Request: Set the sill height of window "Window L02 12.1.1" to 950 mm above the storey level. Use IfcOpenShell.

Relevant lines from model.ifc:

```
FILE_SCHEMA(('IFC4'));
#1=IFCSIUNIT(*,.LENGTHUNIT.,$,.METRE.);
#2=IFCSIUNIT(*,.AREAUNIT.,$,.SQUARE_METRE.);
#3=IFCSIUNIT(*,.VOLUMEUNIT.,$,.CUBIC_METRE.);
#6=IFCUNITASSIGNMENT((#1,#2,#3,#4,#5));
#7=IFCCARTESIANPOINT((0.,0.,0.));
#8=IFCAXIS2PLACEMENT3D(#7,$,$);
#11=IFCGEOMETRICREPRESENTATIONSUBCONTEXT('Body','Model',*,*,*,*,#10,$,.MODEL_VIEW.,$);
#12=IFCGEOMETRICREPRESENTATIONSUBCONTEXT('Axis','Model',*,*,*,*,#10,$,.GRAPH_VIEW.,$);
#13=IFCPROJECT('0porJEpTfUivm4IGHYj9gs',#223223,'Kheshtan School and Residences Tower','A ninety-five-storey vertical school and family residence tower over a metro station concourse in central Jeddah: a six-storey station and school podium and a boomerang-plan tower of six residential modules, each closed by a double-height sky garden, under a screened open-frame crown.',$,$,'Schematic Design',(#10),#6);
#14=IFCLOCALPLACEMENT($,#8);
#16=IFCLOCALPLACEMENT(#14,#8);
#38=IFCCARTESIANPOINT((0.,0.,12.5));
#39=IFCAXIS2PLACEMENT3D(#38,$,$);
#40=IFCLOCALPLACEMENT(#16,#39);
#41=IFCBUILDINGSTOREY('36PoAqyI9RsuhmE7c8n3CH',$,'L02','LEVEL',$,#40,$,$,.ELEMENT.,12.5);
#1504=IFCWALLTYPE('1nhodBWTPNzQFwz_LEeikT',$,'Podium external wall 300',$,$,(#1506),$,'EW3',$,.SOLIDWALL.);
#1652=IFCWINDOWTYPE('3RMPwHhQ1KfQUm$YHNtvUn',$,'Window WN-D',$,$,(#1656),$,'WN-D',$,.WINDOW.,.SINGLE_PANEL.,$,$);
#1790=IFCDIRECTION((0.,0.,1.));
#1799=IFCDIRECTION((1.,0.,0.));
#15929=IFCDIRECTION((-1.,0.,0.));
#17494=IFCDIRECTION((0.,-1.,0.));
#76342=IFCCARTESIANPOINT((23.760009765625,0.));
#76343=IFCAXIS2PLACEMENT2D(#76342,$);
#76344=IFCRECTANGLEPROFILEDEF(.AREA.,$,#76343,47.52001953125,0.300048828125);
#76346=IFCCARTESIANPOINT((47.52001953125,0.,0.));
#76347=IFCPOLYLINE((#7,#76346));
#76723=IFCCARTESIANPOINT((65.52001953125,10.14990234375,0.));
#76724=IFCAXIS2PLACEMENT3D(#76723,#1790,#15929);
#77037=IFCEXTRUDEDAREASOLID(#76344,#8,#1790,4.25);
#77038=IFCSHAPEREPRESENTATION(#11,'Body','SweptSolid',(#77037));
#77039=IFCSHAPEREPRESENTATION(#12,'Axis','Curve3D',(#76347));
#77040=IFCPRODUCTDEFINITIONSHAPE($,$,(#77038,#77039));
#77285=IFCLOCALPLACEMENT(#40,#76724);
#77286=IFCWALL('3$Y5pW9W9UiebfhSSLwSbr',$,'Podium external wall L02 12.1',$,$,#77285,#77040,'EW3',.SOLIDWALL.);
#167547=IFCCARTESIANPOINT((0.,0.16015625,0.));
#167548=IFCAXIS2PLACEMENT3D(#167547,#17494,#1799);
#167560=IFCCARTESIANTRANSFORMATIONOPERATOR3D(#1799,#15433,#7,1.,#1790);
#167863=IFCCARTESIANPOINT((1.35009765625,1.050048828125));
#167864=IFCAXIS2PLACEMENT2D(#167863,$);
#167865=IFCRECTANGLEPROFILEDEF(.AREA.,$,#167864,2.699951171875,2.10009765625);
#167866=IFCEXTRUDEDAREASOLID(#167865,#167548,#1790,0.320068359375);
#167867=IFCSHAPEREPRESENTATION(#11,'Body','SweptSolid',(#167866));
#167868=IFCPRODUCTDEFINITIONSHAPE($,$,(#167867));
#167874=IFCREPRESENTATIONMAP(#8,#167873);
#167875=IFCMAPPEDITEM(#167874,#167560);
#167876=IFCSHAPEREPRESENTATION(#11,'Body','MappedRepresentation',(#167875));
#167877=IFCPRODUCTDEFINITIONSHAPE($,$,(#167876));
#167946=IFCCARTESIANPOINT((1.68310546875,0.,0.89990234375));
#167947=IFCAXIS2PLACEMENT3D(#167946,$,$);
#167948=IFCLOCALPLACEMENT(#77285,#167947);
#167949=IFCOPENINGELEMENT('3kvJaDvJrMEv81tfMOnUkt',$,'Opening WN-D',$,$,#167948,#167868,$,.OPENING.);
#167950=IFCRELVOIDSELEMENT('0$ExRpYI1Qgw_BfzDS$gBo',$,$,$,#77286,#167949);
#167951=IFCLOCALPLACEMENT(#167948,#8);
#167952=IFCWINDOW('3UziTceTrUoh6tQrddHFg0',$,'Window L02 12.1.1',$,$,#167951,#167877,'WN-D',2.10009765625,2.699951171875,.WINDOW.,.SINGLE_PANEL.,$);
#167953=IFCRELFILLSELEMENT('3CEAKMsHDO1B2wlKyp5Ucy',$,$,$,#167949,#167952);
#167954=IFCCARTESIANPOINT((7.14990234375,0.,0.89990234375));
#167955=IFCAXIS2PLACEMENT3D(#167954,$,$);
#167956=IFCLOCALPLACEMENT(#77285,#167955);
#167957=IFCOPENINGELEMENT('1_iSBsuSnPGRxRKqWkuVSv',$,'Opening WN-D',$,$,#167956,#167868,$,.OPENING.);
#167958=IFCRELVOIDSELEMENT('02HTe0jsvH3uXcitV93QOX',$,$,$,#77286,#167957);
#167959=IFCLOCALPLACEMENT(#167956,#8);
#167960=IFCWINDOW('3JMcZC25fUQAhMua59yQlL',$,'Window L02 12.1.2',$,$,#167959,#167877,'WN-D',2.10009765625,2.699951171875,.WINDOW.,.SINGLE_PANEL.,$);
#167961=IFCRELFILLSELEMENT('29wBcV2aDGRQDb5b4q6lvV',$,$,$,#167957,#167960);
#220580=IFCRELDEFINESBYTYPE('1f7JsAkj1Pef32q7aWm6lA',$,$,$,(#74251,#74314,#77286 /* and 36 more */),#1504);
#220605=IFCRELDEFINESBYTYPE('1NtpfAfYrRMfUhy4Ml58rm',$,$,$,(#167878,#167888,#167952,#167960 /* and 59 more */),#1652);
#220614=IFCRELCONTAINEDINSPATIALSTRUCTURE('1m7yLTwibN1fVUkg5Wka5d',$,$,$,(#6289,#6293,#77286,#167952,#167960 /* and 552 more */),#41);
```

```python
import numpy as np
import ifcopenshell
import ifcopenshell.api.geometry
import ifcopenshell.geom
import ifcopenshell.util.element
import ifcopenshell.util.placement
import ifcopenshell.util.shape
import ifcopenshell.util.unit

model = ifcopenshell.open("model.ifc")
unit_scale = ifcopenshell.util.unit.calculate_unit_scale(model)

window = model.by_guid("3UziTceTrUoh6tQrddHFg0")
opening = window.FillsVoids[0].RelatingOpeningElement
storey = ifcopenshell.util.element.get_container(window, ifc_class="IfcBuildingStorey")
level = ifcopenshell.util.placement.get_local_placement(storey.ObjectPlacement)[2, 3]

# The opening's origin need not be at the sill, so measure its lowest point.
shape = ifcopenshell.geom.create_shape(ifcopenshell.geom.settings(), opening)
bottom = ifcopenshell.util.shape.get_shape_bottom_elevation(shape, shape.geometry) / unit_scale
dz = level + 0.95 / unit_scale - bottom

shift = np.array([0.0, 0.0, dz])
# The window is placed relative to its opening, so it follows when the opening moves.
matrix = ifcopenshell.util.placement.get_local_placement(opening.ObjectPlacement)
matrix[:3, 3] += shift
ifcopenshell.api.geometry.edit_object_placement(
    model, product=opening, matrix=matrix, is_si=False, should_transform_children=True
)

print(f"moved by {dz * unit_scale:+.3f} m")

model.write("model_rev.ifc")
```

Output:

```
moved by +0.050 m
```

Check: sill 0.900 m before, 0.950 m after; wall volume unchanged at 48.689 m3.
